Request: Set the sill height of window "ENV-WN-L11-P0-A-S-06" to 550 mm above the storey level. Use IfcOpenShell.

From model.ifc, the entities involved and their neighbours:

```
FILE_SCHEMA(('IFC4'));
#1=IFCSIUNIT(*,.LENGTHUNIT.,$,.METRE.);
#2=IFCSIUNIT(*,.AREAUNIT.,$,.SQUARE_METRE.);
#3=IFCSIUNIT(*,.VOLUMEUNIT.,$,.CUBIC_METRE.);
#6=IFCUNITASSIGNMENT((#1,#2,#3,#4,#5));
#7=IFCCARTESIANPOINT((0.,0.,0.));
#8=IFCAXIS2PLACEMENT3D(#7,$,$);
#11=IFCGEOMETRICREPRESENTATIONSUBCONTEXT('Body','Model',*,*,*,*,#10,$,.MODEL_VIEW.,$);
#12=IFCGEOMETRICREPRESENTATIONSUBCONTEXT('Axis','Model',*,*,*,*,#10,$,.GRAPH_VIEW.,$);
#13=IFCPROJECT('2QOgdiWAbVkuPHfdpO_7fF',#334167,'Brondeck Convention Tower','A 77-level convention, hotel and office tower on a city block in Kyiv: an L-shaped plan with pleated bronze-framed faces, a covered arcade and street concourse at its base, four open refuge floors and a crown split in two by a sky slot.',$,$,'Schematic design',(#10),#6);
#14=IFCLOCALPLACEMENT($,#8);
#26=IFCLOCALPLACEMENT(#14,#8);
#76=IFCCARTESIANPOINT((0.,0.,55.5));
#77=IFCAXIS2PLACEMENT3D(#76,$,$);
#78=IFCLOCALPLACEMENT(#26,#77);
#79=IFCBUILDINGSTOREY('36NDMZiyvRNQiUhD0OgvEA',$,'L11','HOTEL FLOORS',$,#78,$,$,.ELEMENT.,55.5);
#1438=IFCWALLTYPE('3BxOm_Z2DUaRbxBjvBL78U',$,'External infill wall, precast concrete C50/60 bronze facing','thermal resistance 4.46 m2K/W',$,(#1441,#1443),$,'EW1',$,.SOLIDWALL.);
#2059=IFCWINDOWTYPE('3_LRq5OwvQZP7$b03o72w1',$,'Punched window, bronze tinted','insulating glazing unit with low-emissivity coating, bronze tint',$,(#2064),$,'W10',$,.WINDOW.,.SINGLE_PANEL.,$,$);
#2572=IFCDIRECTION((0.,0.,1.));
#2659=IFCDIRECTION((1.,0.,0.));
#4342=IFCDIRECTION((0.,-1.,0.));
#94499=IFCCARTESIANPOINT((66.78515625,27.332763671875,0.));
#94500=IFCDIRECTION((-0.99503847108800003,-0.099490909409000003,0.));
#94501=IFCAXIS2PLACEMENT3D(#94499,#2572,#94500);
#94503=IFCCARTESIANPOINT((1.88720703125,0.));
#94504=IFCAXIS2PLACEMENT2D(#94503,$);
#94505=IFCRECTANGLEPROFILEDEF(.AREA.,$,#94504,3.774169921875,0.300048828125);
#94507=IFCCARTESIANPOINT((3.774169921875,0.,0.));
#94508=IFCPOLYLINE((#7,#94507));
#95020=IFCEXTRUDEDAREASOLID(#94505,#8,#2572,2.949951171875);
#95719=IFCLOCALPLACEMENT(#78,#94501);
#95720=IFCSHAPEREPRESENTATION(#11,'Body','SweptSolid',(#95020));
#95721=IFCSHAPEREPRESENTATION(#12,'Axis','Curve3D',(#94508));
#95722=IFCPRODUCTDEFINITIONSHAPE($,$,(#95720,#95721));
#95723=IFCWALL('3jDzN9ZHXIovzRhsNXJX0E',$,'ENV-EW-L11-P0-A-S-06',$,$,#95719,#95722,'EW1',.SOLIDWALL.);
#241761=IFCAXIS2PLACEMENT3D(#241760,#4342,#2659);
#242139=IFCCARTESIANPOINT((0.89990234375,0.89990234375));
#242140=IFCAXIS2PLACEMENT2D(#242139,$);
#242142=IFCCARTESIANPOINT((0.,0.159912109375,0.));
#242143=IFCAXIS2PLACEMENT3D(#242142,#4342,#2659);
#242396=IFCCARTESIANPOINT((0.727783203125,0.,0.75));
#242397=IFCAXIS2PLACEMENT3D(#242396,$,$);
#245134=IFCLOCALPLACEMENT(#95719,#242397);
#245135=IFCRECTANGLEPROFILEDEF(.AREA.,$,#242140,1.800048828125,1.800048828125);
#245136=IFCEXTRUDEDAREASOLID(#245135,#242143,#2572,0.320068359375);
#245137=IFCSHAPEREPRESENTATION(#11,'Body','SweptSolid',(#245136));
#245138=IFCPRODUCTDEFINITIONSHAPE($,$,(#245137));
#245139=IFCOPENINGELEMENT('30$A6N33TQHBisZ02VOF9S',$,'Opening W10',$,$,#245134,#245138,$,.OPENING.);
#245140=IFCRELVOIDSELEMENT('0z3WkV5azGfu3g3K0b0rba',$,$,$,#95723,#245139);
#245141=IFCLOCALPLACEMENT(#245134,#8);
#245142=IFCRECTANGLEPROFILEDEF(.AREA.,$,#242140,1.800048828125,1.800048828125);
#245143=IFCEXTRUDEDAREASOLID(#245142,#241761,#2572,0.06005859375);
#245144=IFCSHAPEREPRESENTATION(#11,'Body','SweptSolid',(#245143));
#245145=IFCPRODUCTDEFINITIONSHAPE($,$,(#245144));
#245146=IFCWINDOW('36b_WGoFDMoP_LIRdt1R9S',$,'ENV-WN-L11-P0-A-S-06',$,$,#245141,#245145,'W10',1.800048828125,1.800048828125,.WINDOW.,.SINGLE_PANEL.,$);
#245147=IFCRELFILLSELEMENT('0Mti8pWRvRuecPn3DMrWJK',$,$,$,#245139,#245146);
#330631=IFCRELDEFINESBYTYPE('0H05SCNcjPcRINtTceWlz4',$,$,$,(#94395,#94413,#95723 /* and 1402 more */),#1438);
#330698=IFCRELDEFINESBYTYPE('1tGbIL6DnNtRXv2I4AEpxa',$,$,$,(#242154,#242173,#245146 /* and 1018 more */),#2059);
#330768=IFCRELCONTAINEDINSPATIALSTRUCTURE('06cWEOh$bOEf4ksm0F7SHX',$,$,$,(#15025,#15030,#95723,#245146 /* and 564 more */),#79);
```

```python
import numpy as np
import ifcopenshell
import ifcopenshell.api.geometry
import ifcopenshell.geom
import ifcopenshell.util.element
import ifcopenshell.util.placement
import ifcopenshell.util.shape
import ifcopenshell.util.unit

model = ifcopenshell.open("model.ifc")
unit_scale = ifcopenshell.util.unit.calculate_unit_scale(model)

window = model.by_guid("36b_WGoFDMoP_LIRdt1R9S")
opening = window.FillsVoids[0].RelatingOpeningElement
storey = ifcopenshell.util.element.get_container(window, ifc_class="IfcBuildingStorey")
level = ifcopenshell.util.placement.get_local_placement(storey.ObjectPlacement)[2, 3]

# The opening's origin need not be at the sill, so measure its lowest point.
shape = ifcopenshell.geom.create_shape(ifcopenshell.geom.settings(), opening)
bottom = ifcopenshell.util.shape.get_shape_bottom_elevation(shape, shape.geometry) / unit_scale
dz = level + 0.55 - bottom

shift = np.array([0.0, 0.0, dz])
# The window is placed relative to its opening, so it follows when the opening moves.
matrix = ifcopenshell.util.placement.get_local_placement(opening.ObjectPlacement)
matrix[:3, 3] += shift
ifcopenshell.api.geometry.edit_object_placement(
    model, product=opening, matrix=matrix, is_si=False, should_transform_children=True
)

print(f"moved by {dz * unit_scale:+.3f} m")

model.write("model_edited.ifc")
```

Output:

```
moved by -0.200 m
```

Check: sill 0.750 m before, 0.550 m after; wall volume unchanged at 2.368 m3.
